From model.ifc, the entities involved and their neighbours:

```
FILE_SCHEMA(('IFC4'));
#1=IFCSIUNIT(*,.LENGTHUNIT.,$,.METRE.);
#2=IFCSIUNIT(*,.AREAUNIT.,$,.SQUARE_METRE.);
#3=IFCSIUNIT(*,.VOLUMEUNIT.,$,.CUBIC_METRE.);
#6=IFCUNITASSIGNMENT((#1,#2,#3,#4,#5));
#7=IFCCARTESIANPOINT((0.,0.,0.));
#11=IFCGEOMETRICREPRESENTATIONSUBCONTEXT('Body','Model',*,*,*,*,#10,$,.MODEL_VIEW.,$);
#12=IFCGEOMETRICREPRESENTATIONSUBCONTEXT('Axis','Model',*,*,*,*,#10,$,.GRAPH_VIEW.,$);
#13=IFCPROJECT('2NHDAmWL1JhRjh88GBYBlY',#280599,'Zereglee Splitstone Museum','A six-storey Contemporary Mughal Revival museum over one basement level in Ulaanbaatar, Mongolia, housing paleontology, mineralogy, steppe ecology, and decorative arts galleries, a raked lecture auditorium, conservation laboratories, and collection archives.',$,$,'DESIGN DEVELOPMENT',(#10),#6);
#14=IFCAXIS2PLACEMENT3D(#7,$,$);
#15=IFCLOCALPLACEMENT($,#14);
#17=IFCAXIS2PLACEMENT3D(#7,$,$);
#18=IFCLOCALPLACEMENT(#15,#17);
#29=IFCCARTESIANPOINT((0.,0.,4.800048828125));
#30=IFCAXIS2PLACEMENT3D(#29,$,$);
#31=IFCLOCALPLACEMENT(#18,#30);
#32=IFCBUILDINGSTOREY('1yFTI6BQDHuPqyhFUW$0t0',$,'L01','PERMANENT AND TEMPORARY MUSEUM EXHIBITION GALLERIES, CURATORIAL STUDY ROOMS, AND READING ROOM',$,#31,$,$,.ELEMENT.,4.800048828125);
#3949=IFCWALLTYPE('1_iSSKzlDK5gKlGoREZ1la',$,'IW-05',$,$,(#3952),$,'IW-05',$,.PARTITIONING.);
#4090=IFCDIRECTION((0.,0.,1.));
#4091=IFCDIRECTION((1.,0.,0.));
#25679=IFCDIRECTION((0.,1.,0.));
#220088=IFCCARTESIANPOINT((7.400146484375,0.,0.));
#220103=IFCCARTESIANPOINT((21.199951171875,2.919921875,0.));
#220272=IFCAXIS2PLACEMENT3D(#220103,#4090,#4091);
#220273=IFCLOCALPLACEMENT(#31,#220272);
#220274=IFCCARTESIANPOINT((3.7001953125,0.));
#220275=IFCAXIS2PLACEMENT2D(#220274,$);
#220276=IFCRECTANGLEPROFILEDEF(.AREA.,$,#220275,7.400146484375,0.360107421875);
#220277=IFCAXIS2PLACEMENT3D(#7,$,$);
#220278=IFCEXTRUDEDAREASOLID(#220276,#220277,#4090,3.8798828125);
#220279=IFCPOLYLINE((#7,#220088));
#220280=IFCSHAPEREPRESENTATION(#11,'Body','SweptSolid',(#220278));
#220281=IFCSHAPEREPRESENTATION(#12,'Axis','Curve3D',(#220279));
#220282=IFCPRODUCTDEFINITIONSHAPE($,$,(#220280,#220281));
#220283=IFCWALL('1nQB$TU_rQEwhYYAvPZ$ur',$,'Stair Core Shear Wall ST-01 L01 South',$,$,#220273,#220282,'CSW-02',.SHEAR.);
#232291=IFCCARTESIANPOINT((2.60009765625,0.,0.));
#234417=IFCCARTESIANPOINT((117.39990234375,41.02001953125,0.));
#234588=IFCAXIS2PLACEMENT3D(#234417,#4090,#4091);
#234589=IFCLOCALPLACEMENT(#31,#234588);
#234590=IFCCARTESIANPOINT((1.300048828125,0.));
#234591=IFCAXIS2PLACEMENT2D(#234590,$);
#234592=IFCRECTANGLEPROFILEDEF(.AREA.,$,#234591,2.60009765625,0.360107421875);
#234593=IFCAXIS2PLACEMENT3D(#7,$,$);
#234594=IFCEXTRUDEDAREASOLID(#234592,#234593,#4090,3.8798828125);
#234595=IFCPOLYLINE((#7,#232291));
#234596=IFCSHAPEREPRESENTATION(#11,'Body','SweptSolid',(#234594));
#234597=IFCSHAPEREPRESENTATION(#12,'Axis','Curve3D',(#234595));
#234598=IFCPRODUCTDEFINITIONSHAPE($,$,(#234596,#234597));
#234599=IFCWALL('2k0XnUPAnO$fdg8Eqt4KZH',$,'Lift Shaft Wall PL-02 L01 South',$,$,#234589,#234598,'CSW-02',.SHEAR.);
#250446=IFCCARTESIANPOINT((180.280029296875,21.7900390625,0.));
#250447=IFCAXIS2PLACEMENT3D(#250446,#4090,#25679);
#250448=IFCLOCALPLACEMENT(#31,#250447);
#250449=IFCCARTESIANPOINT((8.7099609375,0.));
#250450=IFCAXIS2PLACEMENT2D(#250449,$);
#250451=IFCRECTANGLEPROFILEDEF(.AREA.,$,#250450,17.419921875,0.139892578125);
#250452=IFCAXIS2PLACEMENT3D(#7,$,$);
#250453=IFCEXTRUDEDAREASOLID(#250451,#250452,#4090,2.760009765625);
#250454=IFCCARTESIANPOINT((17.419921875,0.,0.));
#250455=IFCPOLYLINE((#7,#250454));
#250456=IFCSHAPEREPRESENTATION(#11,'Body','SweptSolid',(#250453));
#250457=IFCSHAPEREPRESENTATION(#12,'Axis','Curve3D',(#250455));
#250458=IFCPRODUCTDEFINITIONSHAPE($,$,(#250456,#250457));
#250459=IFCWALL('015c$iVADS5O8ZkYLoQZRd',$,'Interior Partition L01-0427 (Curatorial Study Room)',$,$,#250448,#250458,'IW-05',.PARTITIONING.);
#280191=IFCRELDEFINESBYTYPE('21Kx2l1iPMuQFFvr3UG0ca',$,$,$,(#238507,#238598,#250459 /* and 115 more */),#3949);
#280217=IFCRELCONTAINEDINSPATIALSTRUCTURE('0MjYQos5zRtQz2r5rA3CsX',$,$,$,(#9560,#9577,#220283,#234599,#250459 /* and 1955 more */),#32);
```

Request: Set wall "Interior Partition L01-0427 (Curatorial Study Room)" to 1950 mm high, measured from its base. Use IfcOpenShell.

```python
import ifcopenshell
import ifcopenshell.geom
import ifcopenshell.util.representation
import ifcopenshell.util.shape

model = ifcopenshell.open("model.ifc")
settings = ifcopenshell.geom.settings()


def volume(element):
    """Net volume in cubic metres, openings subtracted."""
    shape = ifcopenshell.geom.create_shape(settings, element)
    return ifcopenshell.util.shape.get_volume(shape.geometry)


wall = model.by_id(250459)
before = volume(wall)

body = ifcopenshell.util.representation.get_representation(wall, "Model", "Body")
solid = body.Items[0]
old_height = solid.Depth
solid.Depth = 1.95
after = volume(wall)

print(f"height {old_height:g} -> {solid.Depth:g}, volume {before:.3f} -> {after:.3f} m3")

model.write("model_edited.ifc")
```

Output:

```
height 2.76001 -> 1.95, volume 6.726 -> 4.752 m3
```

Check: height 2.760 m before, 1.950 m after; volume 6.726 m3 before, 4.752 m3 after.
